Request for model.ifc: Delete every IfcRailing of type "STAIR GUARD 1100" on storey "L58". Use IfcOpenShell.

First a look at what the model holds.

```python
import ifcopenshell
import ifcopenshell.util.element

model = ifcopenshell.open("model.ifc")
print(model.schema)
storey = next(s for s in model.by_type("IfcBuildingStorey") if s.Name == "L58")
railings = [e for e in ifcopenshell.util.element.get_decomposition(storey) if e.is_a("IfcRailing")]
seen = {}
for e in railings:
    element_type = ifcopenshell.util.element.get_type(e)
    name = element_type.Name if element_type not in (None, e) else None
    seen[name] = seen.get(name, 0) + 1
for name, count in sorted(seen.items(), key=str):
    print(count, "x", name)
```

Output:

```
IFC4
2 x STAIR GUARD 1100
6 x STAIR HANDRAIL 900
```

```python
import ifcopenshell
import ifcopenshell.api.root
import ifcopenshell.util.element

model = ifcopenshell.open("model.ifc")

storey = next(s for s in model.by_type("IfcBuildingStorey") if s.Name == "L58")
railings = [e for e in ifcopenshell.util.element.get_decomposition(storey) if e.is_a("IfcRailing")]
targets = [e for e in railings if (t := ifcopenshell.util.element.get_type(e)) not in (None, e) and t.Name == "STAIR GUARD 1100"]

for e in targets:
    ifcopenshell.api.root.remove_product(model, product=e)
print(len(targets), "removed")

model.write("model_v2.ifc")
```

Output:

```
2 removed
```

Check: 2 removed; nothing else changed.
